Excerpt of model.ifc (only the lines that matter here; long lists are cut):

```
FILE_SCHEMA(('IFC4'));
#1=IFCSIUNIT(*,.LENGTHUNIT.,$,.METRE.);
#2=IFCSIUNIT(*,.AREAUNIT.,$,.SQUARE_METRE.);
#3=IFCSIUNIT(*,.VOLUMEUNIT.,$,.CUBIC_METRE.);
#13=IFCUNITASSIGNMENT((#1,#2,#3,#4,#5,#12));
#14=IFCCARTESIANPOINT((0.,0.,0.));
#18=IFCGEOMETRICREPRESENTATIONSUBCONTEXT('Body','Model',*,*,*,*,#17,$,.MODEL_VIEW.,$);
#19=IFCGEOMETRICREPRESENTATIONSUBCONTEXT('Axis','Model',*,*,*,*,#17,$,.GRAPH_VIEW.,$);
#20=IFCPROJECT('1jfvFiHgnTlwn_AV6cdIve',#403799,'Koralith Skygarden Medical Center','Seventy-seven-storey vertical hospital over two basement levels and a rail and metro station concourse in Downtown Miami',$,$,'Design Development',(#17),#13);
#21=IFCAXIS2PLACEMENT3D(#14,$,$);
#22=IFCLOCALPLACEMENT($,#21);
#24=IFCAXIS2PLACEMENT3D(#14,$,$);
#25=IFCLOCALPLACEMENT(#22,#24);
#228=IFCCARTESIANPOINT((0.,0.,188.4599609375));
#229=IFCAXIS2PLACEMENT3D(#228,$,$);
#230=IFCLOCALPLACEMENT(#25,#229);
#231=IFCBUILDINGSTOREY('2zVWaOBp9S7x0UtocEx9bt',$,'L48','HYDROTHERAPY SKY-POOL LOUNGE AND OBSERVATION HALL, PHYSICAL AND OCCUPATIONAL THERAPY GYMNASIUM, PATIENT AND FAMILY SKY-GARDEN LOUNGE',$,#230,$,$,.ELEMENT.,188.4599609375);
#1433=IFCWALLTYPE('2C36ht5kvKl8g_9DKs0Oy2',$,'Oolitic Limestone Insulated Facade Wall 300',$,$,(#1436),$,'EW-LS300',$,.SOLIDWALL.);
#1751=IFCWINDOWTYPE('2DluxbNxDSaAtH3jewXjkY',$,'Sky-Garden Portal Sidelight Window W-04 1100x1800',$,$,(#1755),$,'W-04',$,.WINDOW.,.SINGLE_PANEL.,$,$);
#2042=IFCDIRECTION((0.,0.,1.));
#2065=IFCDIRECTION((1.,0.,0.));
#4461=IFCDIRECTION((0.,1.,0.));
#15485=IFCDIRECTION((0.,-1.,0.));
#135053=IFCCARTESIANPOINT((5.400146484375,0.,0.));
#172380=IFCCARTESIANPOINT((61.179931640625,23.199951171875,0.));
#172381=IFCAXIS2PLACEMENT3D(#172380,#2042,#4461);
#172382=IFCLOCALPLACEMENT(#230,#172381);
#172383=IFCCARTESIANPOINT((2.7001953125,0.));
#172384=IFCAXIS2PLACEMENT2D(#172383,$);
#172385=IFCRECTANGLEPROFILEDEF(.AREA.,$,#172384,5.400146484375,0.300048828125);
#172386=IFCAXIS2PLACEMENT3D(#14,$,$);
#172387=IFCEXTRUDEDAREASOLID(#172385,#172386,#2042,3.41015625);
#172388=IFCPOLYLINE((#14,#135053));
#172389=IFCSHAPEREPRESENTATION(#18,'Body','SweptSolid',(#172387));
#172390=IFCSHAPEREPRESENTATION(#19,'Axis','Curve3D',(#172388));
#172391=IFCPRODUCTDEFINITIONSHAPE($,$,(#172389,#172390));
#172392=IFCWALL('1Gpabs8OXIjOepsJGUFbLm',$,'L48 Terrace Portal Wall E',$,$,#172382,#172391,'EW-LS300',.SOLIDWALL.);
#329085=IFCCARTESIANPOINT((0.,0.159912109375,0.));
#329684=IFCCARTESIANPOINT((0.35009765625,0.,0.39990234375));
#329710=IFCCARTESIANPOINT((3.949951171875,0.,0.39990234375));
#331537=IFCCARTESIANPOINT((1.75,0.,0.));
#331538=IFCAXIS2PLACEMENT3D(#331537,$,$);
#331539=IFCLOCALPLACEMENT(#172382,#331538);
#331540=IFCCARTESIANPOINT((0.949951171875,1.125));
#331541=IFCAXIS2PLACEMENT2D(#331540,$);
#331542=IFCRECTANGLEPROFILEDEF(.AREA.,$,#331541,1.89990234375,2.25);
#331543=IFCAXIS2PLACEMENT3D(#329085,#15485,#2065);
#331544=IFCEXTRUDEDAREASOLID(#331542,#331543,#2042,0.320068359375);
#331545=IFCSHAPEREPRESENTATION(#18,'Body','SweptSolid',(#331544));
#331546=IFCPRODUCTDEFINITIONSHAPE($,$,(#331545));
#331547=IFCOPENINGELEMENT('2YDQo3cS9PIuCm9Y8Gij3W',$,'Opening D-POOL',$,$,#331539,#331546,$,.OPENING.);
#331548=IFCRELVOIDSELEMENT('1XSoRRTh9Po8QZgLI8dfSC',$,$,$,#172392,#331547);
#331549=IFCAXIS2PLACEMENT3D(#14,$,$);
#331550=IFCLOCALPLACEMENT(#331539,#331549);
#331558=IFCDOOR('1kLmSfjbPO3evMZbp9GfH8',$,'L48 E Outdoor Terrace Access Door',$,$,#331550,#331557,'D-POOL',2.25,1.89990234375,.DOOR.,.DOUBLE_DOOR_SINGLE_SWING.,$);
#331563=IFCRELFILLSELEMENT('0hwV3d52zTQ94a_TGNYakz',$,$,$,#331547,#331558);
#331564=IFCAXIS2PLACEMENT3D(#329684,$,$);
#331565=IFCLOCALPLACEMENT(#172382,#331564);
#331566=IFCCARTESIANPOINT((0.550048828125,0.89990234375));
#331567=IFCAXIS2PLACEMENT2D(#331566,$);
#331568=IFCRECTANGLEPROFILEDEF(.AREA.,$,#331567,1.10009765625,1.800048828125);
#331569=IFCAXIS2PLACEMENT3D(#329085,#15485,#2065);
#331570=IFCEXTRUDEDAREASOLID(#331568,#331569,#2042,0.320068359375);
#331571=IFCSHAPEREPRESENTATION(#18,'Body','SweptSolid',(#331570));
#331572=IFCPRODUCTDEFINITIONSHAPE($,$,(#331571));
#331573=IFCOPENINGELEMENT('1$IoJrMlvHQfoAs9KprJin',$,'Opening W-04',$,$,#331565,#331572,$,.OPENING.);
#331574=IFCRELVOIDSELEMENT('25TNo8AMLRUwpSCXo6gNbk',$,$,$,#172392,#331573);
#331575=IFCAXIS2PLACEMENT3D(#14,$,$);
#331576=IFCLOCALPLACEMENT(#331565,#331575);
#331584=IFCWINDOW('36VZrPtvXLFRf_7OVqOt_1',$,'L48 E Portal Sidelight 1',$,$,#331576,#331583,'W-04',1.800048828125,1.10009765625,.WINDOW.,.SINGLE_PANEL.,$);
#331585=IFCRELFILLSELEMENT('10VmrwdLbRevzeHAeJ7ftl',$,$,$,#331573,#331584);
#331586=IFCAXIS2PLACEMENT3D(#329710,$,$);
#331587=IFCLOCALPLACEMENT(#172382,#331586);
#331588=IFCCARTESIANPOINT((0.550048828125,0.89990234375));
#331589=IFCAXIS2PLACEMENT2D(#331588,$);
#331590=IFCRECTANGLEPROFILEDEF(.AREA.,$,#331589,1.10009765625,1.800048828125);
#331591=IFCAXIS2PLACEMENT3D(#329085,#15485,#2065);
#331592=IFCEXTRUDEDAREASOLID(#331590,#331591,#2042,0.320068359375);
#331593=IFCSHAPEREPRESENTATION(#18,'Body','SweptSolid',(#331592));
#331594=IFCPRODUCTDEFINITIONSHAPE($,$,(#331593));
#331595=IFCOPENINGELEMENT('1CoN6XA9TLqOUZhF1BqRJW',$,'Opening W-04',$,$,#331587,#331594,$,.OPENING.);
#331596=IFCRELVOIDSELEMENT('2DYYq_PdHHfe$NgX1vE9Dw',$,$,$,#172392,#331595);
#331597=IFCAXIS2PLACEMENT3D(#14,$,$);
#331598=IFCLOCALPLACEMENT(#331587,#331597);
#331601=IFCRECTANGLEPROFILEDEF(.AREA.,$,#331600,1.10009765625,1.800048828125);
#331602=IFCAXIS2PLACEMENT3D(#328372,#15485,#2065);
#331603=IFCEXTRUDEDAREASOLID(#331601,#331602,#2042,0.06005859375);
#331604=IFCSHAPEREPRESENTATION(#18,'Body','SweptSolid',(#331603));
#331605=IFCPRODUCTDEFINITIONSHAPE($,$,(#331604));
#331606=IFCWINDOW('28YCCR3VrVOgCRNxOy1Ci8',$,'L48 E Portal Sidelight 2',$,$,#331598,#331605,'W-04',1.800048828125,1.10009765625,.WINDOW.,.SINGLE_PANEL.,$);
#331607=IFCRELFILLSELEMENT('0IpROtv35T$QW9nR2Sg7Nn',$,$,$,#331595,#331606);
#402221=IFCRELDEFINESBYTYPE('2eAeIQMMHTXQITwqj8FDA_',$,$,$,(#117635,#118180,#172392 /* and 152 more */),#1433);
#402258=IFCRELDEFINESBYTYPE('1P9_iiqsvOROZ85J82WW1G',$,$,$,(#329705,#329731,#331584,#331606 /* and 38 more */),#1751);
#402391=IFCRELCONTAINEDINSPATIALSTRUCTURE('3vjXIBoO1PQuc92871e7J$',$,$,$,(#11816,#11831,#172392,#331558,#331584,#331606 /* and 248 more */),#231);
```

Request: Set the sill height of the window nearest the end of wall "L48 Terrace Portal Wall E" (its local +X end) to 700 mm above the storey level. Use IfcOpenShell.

```python
import numpy as np
import ifcopenshell
import ifcopenshell.api.geometry
import ifcopenshell.geom
import ifcopenshell.util.element
import ifcopenshell.util.placement
import ifcopenshell.util.shape
import ifcopenshell.util.unit

model = ifcopenshell.open("model.ifc")
unit_scale = ifcopenshell.util.unit.calculate_unit_scale(model)

window = model.by_id(331606)
opening = window.FillsVoids[0].RelatingOpeningElement
storey = ifcopenshell.util.element.get_container(window, ifc_class="IfcBuildingStorey")
level = ifcopenshell.util.placement.get_local_placement(storey.ObjectPlacement)[2, 3]

# The opening's origin need not be at the sill, so measure its lowest point.
shape = ifcopenshell.geom.create_shape(ifcopenshell.geom.settings(), opening)
bottom = ifcopenshell.util.shape.get_shape_bottom_elevation(shape, shape.geometry) / unit_scale
dz = level + 0.7 - bottom

shift = np.array([0.0, 0.0, dz])
# The window is placed relative to its opening, so it follows when the opening moves.
matrix = ifcopenshell.util.placement.get_local_placement(opening.ObjectPlacement)
matrix[:3, 3] += shift
ifcopenshell.api.geometry.edit_object_placement(
    model, product=opening, matrix=matrix, is_si=False, should_transform_children=True
)

print(f"moved by {dz * unit_scale:+.3f} m")

model.write("model_updated.ifc")
```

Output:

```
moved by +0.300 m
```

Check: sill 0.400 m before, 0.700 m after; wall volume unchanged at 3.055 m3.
